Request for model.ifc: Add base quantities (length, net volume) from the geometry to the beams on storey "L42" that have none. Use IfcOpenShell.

First a look at what the model holds.

```python
import ifcopenshell
import ifcopenshell.util.element
import ifcopenshell.util.unit

model = ifcopenshell.open("model.ifc")
print(model.schema)
for unit_type in ("LENGTHUNIT", "AREAUNIT", "VOLUMEUNIT"):
    print(unit_type, ifcopenshell.util.unit.calculate_unit_scale(model, unit_type))
storey = next(s for s in model.by_type("IfcBuildingStorey") if s.Name == "L42")
beams = [e for e in ifcopenshell.util.element.get_decomposition(storey) if e.is_a("IfcBeam")]
for e in sorted(beams, key=lambda e: e.id()):
    print(e.id(), e.is_a(), e.Name, list(ifcopenshell.util.element.get_psets(e, qtos_only=True)), sep=" | ")
```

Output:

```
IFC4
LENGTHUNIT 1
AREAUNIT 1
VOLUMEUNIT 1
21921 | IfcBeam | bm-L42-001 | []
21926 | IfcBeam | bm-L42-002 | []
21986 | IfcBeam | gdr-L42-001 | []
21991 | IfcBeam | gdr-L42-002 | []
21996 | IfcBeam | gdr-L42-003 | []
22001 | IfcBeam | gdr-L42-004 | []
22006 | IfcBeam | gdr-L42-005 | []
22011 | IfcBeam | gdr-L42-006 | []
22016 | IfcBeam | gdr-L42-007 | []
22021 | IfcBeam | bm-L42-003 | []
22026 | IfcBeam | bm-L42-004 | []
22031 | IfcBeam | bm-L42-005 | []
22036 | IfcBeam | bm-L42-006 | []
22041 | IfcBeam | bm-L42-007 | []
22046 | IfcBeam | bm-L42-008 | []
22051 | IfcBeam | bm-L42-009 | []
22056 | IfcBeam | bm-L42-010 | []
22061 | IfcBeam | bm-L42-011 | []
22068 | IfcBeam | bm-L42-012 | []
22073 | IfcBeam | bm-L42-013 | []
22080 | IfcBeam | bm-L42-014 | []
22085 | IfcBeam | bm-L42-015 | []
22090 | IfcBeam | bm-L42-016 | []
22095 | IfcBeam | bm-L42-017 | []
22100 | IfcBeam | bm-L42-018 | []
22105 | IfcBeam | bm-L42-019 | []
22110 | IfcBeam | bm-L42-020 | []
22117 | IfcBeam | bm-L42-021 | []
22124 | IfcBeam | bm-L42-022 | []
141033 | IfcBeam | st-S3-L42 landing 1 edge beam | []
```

```python
import ifcopenshell
import ifcopenshell.api.pset
import ifcopenshell.geom
import ifcopenshell.util.element
import ifcopenshell.util.shape
import ifcopenshell.util.unit

model = ifcopenshell.open("model.ifc")
unit_scale = ifcopenshell.util.unit.calculate_unit_scale(model)
volume_scale = ifcopenshell.util.unit.calculate_unit_scale(model, "VOLUMEUNIT")
settings = ifcopenshell.geom.settings()

storey = next(s for s in model.by_type("IfcBuildingStorey") if s.Name == "L42")
beams = [e for e in ifcopenshell.util.element.get_decomposition(storey) if e.is_a("IfcBeam")]

for e in sorted(beams, key=lambda e: e.id()):
    if ifcopenshell.util.element.get_psets(e, qtos_only=True, should_inherit=False):
        continue
    # Geometry comes back in metres, in the element's own axes.
    shape = ifcopenshell.geom.create_shape(settings, e)
    values = {
        "Length": ifcopenshell.util.shape.get_max_xyz(shape.geometry) / unit_scale,
        "NetVolume": ifcopenshell.util.shape.get_volume(shape.geometry) / volume_scale,
    }
    qto = ifcopenshell.api.pset.add_qto(model, product=e, name="Qto_BeamBaseQuantities")
    ifcopenshell.api.pset.edit_qto(model, qto=qto, properties=values)
    print(e.id(), {k: round(v, 3) for k, v in values.items()})

model.write("model-out.ifc")
```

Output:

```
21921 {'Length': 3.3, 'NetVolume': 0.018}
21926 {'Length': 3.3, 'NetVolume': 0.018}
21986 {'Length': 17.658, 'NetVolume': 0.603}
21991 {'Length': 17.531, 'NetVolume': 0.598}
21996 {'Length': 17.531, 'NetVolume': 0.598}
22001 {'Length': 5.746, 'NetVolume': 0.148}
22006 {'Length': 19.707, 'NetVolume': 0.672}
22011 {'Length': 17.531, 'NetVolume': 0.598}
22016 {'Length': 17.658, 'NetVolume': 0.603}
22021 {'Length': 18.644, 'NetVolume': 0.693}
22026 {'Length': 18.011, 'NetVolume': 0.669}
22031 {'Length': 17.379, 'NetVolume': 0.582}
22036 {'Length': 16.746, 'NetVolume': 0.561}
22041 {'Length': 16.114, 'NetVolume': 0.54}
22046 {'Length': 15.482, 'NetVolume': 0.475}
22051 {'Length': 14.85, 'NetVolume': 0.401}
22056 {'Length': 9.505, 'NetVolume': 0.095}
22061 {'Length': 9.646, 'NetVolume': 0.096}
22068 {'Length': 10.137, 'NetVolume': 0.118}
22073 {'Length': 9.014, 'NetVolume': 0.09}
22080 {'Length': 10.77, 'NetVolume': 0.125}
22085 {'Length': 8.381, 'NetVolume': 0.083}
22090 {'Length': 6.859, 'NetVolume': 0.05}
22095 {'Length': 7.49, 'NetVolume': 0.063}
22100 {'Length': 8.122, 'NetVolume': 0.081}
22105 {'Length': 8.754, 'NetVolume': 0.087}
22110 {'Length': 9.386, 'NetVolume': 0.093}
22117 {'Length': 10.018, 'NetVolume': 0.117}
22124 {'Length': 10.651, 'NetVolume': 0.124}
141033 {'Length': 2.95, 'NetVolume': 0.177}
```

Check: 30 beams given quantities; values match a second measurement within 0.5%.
